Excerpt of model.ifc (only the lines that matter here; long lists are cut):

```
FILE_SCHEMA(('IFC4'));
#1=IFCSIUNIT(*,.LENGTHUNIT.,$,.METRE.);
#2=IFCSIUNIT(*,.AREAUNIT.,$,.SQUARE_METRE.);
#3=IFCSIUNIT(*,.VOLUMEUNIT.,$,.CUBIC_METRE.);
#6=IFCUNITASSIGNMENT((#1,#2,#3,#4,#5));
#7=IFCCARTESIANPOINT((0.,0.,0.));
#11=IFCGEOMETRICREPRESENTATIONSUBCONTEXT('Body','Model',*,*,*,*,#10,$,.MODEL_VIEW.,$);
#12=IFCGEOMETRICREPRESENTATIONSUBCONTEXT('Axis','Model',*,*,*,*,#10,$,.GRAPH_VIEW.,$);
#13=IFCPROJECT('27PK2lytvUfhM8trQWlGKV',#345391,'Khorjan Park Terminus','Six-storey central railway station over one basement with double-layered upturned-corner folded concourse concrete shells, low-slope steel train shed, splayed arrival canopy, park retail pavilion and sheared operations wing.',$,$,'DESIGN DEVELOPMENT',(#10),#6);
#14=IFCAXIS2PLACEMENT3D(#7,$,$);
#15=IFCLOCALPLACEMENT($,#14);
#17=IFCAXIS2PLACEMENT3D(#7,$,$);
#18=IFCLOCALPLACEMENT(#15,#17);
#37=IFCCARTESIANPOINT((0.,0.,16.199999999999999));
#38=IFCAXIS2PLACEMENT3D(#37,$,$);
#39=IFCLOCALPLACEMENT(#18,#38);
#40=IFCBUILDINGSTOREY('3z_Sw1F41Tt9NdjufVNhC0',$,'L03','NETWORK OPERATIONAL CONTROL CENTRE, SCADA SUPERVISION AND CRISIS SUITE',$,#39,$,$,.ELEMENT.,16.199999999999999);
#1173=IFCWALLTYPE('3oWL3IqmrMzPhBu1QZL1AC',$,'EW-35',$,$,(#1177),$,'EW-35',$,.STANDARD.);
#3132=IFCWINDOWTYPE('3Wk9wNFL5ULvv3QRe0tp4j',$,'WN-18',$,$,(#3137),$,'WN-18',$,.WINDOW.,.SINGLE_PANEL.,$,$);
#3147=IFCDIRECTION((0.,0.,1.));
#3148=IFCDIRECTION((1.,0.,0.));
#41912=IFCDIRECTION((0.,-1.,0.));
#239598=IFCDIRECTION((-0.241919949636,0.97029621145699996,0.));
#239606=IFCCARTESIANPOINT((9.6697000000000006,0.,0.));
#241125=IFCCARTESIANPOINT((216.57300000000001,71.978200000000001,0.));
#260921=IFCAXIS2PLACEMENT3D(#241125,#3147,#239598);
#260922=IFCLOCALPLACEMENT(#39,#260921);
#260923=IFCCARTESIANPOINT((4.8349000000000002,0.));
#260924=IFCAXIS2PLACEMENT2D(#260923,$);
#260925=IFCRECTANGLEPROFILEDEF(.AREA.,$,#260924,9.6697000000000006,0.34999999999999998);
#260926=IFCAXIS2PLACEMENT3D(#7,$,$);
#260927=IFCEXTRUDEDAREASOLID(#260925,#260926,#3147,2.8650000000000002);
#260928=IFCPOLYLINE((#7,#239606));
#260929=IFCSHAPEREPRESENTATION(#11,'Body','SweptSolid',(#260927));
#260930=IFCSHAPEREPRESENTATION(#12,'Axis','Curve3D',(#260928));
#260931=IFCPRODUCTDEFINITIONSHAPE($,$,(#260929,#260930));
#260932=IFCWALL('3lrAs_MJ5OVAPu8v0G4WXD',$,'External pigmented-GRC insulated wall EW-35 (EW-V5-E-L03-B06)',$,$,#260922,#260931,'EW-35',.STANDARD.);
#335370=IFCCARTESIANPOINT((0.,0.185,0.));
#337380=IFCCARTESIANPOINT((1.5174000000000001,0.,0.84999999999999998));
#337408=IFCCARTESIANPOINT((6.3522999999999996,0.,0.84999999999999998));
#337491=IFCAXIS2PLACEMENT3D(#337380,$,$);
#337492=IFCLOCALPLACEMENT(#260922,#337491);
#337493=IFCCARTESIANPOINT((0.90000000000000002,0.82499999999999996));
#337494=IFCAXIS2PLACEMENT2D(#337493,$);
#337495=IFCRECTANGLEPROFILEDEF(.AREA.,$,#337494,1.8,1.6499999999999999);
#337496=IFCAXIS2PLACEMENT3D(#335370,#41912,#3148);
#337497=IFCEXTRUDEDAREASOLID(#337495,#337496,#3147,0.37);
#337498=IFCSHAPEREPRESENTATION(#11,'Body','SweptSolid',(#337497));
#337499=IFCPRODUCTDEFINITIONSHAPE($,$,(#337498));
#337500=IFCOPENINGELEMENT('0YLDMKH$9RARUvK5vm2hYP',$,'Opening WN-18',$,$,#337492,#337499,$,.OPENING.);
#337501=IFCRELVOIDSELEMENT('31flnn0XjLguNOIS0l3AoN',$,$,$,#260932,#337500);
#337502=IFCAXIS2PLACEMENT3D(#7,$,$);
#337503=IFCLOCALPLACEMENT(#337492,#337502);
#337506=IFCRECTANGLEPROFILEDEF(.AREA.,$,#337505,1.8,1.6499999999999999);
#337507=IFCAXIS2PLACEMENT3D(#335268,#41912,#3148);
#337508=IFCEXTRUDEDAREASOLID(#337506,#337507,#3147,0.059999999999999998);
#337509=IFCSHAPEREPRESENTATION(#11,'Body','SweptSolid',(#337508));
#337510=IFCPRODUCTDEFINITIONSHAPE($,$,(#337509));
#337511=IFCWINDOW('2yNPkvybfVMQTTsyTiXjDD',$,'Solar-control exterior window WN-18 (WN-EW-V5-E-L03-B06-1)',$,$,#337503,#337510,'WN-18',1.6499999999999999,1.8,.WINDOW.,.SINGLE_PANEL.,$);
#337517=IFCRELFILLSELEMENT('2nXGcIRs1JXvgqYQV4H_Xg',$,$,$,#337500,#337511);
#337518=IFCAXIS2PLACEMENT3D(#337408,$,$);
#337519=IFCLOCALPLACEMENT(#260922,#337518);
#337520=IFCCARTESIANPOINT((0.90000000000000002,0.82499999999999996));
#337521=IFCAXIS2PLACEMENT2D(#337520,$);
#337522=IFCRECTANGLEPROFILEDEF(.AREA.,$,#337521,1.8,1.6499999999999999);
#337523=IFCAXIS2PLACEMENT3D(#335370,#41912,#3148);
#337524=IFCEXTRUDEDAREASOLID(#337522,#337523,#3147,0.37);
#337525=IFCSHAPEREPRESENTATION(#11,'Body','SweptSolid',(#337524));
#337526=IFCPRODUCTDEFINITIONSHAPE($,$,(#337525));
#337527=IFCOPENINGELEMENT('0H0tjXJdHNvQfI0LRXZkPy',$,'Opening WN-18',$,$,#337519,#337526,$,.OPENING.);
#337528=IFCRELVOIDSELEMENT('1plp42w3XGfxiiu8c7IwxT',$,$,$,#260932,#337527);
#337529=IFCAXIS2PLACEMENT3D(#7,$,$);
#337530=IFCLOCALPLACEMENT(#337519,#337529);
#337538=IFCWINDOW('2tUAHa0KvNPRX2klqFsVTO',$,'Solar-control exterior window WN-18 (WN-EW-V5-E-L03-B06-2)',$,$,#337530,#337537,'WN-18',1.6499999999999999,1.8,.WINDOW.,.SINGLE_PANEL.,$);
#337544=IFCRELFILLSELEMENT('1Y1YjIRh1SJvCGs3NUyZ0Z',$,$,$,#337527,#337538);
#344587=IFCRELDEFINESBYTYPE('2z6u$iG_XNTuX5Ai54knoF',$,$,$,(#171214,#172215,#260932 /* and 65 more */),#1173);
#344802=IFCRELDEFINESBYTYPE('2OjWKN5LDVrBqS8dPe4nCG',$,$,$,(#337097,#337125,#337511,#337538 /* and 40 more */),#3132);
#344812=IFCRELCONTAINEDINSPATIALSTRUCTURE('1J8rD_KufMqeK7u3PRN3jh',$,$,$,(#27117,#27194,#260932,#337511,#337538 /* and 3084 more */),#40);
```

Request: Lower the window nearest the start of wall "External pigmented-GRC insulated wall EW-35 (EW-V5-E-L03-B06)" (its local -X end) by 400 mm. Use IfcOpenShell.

```python
import numpy as np
import ifcopenshell
import ifcopenshell.api.geometry
import ifcopenshell.util.placement
import ifcopenshell.util.unit

model = ifcopenshell.open("model.ifc")
unit_scale = ifcopenshell.util.unit.calculate_unit_scale(model)

window = model.by_guid("2yNPkvybfVMQTTsyTiXjDD")
opening = window.FillsVoids[0].RelatingOpeningElement
dz = -0.4 / unit_scale

shift = np.array([0.0, 0.0, dz])
# The window is placed relative to its opening, so it follows when the opening moves.
matrix = ifcopenshell.util.placement.get_local_placement(opening.ObjectPlacement)
matrix[:3, 3] += shift
ifcopenshell.api.geometry.edit_object_placement(
    model, product=opening, matrix=matrix, is_si=False, should_transform_children=True
)

print(f"moved by {dz * unit_scale:+.3f} m")

model.write("model_rev.ifc")
```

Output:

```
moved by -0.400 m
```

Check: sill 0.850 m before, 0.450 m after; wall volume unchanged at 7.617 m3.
